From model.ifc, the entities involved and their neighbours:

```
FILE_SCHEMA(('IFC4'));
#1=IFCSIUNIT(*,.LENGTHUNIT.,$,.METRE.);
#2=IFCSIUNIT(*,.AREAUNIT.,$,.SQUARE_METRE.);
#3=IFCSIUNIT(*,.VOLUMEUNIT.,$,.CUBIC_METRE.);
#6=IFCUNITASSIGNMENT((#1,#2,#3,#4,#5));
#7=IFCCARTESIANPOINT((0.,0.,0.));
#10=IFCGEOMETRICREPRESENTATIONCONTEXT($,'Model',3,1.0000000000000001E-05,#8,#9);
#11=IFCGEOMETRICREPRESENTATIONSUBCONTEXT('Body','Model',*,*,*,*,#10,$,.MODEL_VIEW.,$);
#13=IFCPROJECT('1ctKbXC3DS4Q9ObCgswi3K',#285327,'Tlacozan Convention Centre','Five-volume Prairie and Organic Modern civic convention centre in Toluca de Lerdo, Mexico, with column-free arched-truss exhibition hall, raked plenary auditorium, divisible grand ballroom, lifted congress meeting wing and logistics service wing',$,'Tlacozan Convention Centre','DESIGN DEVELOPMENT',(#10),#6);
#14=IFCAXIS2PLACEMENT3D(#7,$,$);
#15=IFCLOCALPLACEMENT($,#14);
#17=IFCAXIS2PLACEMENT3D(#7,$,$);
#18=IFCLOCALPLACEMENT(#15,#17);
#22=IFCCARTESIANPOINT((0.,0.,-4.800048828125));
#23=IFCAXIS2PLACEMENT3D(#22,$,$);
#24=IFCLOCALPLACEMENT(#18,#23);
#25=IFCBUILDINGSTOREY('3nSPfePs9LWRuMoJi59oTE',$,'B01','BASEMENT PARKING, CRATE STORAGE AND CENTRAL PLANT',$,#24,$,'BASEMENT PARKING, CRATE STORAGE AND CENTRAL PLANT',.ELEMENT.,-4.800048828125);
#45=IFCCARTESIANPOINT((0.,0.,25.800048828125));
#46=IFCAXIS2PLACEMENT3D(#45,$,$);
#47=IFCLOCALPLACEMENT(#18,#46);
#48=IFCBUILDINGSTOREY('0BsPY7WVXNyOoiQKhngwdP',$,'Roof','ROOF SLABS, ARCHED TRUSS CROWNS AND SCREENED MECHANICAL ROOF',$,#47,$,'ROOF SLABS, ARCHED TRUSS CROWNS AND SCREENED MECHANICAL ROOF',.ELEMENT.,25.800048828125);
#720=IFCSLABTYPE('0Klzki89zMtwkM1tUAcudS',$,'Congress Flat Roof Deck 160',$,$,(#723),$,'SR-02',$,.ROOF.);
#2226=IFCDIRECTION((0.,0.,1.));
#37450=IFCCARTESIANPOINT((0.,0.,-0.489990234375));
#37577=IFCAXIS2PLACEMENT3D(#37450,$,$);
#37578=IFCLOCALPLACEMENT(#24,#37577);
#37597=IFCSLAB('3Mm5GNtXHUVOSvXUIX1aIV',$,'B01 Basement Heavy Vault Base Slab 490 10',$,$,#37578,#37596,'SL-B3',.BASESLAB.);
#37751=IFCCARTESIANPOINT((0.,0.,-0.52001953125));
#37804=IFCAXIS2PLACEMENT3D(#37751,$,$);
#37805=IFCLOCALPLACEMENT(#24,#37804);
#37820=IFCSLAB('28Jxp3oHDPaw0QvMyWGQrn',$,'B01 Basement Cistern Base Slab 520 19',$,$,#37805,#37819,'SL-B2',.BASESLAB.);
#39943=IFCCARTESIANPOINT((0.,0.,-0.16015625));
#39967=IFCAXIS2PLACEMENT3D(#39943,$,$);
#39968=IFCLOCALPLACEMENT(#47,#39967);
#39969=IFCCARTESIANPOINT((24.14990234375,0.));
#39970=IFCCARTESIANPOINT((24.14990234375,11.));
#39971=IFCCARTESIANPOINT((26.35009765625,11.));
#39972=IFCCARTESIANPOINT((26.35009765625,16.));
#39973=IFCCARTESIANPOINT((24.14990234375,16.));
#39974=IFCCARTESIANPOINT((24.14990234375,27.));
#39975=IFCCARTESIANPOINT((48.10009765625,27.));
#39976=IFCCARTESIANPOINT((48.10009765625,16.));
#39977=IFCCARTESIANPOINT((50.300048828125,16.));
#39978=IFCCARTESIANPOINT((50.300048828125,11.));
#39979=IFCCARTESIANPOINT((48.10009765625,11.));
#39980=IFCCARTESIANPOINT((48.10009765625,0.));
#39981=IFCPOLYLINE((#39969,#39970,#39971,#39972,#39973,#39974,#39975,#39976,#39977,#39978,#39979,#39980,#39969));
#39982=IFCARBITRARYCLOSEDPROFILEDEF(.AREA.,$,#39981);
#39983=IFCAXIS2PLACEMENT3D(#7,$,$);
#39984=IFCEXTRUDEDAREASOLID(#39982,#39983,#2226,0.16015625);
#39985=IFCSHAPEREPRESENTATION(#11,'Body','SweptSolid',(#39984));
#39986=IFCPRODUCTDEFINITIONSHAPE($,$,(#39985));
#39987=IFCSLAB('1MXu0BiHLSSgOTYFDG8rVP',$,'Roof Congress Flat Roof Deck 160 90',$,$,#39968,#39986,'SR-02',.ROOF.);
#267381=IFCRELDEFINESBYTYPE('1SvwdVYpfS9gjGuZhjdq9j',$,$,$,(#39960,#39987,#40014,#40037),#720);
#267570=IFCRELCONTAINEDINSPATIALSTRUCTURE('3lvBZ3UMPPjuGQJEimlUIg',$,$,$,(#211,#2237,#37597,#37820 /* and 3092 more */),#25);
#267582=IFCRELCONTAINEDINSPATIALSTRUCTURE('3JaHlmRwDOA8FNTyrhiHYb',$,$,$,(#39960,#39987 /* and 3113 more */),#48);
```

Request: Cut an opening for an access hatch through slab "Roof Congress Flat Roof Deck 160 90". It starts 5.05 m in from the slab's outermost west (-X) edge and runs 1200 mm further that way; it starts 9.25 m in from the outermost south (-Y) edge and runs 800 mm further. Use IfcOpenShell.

```python
import numpy as np
import ifcopenshell
import ifcopenshell.api.feature
import ifcopenshell.api.geometry
import ifcopenshell.api.root
import ifcopenshell.geom
import ifcopenshell.util.placement
import ifcopenshell.util.representation
import ifcopenshell.util.shape
import ifcopenshell.util.unit

model = ifcopenshell.open("model.ifc")
unit_scale = ifcopenshell.util.unit.calculate_unit_scale(model)
settings = ifcopenshell.geom.settings()


def volume(element):
    """Net volume in cubic metres, openings subtracted."""
    shape = ifcopenshell.geom.create_shape(settings, element)
    return ifcopenshell.util.shape.get_volume(shape.geometry)


slab = model.by_guid("1MXu0BiHLSSgOTYFDG8rVP")
before = volume(slab)

# Extent in the slab's own axes, in metres. The edges named are its -X and -Y sides.
slab_shape = ifcopenshell.geom.create_shape(settings, slab)
vertices = ifcopenshell.util.shape.get_vertices(slab_shape.geometry)
x_min, y_min, bottom = vertices.min(axis=0)
top = vertices[:, 2].max()

opening = ifcopenshell.api.root.create_entity(model, ifc_class="IfcOpeningElement", name="Access hatch opening", predefined_type="OPENING")
context = ifcopenshell.util.representation.get_context(model, "Model", "Body", "MODEL_VIEW")
width, depth = 1.2, 0.8
outline = [(0.0, 0.0), (width, 0.0), (width, depth), (0.0, depth), (0.0, 0.0)]
# Overshoot both faces by 50 mm so the cut is clean.
shape = ifcopenshell.api.geometry.add_slab_representation(
    model, context=context, depth=top - bottom + 0.1, polyline=outline
)
ifcopenshell.api.geometry.assign_representation(model, product=opening, representation=shape)

matrix = ifcopenshell.util.placement.get_local_placement(slab.ObjectPlacement)
matrix[:, 3] = matrix @ np.append(np.array([x_min + 5.05, y_min + 9.25, bottom - 0.05]) / unit_scale, 1.0)
ifcopenshell.api.geometry.edit_object_placement(model, product=opening, matrix=matrix, is_si=False)
ifcopenshell.api.feature.add_feature(model, feature=opening, element=slab)

after = volume(slab)

print(f"slab volume {before:.3f} -> {after:.3f} m3")

model.write("model-out.ifc")
```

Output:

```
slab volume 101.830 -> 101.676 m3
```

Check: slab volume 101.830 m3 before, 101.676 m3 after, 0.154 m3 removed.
